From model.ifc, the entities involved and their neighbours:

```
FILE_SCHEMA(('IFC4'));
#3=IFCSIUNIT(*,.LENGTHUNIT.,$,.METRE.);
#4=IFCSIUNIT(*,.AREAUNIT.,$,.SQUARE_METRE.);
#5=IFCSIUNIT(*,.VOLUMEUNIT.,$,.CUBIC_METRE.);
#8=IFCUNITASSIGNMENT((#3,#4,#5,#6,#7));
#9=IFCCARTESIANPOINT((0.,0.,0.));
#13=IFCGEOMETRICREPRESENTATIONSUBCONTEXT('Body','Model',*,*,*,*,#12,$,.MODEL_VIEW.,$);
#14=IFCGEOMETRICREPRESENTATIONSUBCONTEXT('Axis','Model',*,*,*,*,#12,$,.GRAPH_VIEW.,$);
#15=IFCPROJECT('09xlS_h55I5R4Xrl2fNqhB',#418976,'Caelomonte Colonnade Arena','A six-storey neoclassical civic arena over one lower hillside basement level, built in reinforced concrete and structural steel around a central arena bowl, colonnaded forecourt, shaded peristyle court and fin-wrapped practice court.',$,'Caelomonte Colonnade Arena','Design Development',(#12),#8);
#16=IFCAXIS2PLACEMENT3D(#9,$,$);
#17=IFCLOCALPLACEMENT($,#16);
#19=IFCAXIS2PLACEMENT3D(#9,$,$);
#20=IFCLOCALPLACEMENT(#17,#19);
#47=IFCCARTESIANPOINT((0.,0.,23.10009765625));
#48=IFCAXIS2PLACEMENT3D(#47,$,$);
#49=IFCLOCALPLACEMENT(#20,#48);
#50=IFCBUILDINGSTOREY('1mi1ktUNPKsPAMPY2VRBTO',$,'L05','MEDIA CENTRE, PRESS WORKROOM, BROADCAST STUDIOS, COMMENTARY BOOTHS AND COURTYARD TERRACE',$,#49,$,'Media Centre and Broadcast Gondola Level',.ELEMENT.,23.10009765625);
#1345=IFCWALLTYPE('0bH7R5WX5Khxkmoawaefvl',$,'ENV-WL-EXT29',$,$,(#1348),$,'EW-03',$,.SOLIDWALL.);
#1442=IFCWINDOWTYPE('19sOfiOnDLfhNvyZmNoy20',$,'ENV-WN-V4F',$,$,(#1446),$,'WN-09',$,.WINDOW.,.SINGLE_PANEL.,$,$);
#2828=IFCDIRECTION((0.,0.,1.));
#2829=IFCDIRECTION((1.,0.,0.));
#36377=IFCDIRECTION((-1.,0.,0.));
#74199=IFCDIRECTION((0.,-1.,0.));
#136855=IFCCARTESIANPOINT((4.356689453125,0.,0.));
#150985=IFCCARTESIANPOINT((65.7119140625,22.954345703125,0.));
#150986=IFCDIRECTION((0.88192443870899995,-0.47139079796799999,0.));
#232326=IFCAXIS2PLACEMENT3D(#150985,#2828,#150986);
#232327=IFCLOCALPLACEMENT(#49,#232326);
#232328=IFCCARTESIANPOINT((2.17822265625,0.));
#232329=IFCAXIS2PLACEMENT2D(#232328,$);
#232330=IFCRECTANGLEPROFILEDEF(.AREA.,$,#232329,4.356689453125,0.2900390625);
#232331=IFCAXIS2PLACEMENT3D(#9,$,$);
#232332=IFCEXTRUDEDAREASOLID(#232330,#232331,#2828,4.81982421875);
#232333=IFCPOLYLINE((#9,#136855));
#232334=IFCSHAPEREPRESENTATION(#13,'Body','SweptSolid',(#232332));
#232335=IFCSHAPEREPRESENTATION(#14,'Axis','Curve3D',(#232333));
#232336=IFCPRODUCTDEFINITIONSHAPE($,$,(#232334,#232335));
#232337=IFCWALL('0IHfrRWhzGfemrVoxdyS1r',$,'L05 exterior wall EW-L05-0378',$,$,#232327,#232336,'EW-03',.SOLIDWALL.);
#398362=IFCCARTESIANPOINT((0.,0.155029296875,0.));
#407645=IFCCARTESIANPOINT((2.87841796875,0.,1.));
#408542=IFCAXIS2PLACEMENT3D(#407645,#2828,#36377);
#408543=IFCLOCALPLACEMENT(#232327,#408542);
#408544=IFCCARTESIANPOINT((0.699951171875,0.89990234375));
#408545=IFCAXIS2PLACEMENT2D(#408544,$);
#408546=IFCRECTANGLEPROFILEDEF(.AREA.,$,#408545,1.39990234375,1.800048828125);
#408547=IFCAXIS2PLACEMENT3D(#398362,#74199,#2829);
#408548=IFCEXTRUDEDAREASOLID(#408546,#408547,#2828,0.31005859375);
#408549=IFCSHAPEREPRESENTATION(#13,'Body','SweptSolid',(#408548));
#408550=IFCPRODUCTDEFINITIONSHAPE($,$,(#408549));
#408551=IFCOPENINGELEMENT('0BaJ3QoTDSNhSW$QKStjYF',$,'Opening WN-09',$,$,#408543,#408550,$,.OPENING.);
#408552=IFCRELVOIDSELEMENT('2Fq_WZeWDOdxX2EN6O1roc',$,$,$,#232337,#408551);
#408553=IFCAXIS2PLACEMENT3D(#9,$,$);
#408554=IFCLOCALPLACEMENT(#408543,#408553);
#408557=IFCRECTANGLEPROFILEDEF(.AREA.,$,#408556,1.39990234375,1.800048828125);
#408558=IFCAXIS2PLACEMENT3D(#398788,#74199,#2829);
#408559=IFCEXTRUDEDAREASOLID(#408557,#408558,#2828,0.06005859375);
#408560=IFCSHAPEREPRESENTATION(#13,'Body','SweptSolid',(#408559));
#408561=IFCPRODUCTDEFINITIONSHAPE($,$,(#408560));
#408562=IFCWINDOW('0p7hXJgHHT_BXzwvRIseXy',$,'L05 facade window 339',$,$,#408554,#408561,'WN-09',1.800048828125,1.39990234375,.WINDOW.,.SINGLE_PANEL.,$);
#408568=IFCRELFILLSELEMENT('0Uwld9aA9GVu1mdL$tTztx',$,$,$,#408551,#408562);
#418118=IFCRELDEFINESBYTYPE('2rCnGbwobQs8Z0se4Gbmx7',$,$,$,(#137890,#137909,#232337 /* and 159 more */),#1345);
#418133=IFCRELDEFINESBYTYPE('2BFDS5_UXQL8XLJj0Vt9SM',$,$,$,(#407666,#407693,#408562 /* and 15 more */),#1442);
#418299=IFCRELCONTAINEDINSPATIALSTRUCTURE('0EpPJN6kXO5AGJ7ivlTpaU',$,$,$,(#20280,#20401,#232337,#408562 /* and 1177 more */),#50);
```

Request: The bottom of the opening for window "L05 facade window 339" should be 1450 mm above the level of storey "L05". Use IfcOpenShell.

```python
import numpy as np
import ifcopenshell
import ifcopenshell.api.geometry
import ifcopenshell.geom
import ifcopenshell.util.element
import ifcopenshell.util.placement
import ifcopenshell.util.shape
import ifcopenshell.util.unit

model = ifcopenshell.open("model.ifc")
unit_scale = ifcopenshell.util.unit.calculate_unit_scale(model)

window = model.by_guid("0p7hXJgHHT_BXzwvRIseXy")
opening = window.FillsVoids[0].RelatingOpeningElement
storey = ifcopenshell.util.element.get_container(window, ifc_class="IfcBuildingStorey")
level = ifcopenshell.util.placement.get_local_placement(storey.ObjectPlacement)[2, 3]

# The opening's origin need not be at the sill, so measure its lowest point.
shape = ifcopenshell.geom.create_shape(ifcopenshell.geom.settings(), opening)
bottom = ifcopenshell.util.shape.get_shape_bottom_elevation(shape, shape.geometry) / unit_scale
dz = level + 1.45 / unit_scale - bottom

shift = np.array([0.0, 0.0, dz])
# The window is placed relative to its opening, so it follows when the opening moves.
matrix = ifcopenshell.util.placement.get_local_placement(opening.ObjectPlacement)
matrix[:3, 3] += shift
ifcopenshell.api.geometry.edit_object_placement(
    model, product=opening, matrix=matrix, is_si=False, should_transform_children=True
)

print(f"moved by {dz * unit_scale:+.3f} m")

model.write("model-out.ifc")
```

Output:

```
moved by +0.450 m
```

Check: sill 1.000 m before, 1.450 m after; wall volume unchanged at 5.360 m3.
